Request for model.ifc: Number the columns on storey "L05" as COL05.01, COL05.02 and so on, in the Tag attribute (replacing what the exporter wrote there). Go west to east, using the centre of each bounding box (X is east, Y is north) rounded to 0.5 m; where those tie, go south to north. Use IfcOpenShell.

First a look at what the model holds.

```python
import ifcopenshell
import ifcopenshell.util.element
import ifcopenshell.util.placement

model = ifcopenshell.open("model.ifc")
print(model.schema)
storey = next(s for s in model.by_type("IfcBuildingStorey") if s.Name == "L05")
columns = [e for e in ifcopenshell.util.element.get_decomposition(storey) if e.is_a("IfcColumn")]
for e in sorted(columns, key=lambda e: e.id()):
    origin = ifcopenshell.util.placement.get_local_placement(e.ObjectPlacement)[:3, 3]
    print(e.id(), e.Tag, e.Name, origin.round(2) + 0.0, sep=" | ")
```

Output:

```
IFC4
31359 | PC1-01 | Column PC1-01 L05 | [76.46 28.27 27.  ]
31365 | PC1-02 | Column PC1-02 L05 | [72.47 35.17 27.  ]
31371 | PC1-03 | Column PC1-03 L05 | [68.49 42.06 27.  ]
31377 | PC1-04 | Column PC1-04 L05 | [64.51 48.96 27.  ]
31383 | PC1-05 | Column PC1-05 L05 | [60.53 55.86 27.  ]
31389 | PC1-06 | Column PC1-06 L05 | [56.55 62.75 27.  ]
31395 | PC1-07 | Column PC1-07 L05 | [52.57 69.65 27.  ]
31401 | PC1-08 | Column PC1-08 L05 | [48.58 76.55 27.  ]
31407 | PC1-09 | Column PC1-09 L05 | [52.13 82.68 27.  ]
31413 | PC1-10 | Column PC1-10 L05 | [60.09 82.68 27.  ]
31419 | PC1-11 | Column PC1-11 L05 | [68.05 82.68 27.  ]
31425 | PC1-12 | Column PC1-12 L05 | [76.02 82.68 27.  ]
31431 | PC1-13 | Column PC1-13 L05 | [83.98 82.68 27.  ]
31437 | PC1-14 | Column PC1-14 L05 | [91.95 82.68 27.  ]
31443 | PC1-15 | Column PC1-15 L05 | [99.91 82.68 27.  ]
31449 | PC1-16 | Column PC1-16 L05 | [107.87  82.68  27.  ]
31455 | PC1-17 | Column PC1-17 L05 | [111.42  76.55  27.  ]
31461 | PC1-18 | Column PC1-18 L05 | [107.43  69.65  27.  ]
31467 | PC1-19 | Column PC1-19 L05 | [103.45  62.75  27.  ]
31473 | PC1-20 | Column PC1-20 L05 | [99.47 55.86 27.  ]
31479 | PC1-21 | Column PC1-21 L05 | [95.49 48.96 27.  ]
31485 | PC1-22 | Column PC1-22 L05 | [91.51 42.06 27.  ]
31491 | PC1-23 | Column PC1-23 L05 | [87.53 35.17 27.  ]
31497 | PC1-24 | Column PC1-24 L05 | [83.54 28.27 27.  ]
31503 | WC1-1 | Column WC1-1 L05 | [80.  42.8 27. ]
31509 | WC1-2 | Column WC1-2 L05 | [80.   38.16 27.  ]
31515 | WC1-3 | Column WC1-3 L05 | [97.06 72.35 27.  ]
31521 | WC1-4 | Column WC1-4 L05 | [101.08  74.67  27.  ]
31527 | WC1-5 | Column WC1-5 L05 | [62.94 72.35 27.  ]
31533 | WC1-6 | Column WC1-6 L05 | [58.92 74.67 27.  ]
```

```python
import ifcopenshell
import ifcopenshell.geom
import ifcopenshell.util.element
import ifcopenshell.util.shape

model = ifcopenshell.open("model.ifc")
settings = ifcopenshell.geom.settings()
settings.set("use-world-coords", True)


def centre(element):
    shape = ifcopenshell.geom.create_shape(settings, element)
    return ifcopenshell.util.shape.get_bbox_centroid(shape.geometry)


storey = next(s for s in model.by_type("IfcBuildingStorey") if s.Name == "L05")
columns = [e for e in ifcopenshell.util.element.get_decomposition(storey) if e.is_a("IfcColumn")]

# Insertion points can sit at a corner or the storey origin, so sort by the geometry (in metres).
centres = {e: centre(e) for e in columns}
columns.sort(key=lambda e: (round(centres[e][0] / 0.5), centres[e][1]))

for i, e in enumerate(columns, start=1):
    number = f"COL05.{i:02d}"
    e.Tag = number
    print(e.id(), number)

model.write("model_v2.ifc")
```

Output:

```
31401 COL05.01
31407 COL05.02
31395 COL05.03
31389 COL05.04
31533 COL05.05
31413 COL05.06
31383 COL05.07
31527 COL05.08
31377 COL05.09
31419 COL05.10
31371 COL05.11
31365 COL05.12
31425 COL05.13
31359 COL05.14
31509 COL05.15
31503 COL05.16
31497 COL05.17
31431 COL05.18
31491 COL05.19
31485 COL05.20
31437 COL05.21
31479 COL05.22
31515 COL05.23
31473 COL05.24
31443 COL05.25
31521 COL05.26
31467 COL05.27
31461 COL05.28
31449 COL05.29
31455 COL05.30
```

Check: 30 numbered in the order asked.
